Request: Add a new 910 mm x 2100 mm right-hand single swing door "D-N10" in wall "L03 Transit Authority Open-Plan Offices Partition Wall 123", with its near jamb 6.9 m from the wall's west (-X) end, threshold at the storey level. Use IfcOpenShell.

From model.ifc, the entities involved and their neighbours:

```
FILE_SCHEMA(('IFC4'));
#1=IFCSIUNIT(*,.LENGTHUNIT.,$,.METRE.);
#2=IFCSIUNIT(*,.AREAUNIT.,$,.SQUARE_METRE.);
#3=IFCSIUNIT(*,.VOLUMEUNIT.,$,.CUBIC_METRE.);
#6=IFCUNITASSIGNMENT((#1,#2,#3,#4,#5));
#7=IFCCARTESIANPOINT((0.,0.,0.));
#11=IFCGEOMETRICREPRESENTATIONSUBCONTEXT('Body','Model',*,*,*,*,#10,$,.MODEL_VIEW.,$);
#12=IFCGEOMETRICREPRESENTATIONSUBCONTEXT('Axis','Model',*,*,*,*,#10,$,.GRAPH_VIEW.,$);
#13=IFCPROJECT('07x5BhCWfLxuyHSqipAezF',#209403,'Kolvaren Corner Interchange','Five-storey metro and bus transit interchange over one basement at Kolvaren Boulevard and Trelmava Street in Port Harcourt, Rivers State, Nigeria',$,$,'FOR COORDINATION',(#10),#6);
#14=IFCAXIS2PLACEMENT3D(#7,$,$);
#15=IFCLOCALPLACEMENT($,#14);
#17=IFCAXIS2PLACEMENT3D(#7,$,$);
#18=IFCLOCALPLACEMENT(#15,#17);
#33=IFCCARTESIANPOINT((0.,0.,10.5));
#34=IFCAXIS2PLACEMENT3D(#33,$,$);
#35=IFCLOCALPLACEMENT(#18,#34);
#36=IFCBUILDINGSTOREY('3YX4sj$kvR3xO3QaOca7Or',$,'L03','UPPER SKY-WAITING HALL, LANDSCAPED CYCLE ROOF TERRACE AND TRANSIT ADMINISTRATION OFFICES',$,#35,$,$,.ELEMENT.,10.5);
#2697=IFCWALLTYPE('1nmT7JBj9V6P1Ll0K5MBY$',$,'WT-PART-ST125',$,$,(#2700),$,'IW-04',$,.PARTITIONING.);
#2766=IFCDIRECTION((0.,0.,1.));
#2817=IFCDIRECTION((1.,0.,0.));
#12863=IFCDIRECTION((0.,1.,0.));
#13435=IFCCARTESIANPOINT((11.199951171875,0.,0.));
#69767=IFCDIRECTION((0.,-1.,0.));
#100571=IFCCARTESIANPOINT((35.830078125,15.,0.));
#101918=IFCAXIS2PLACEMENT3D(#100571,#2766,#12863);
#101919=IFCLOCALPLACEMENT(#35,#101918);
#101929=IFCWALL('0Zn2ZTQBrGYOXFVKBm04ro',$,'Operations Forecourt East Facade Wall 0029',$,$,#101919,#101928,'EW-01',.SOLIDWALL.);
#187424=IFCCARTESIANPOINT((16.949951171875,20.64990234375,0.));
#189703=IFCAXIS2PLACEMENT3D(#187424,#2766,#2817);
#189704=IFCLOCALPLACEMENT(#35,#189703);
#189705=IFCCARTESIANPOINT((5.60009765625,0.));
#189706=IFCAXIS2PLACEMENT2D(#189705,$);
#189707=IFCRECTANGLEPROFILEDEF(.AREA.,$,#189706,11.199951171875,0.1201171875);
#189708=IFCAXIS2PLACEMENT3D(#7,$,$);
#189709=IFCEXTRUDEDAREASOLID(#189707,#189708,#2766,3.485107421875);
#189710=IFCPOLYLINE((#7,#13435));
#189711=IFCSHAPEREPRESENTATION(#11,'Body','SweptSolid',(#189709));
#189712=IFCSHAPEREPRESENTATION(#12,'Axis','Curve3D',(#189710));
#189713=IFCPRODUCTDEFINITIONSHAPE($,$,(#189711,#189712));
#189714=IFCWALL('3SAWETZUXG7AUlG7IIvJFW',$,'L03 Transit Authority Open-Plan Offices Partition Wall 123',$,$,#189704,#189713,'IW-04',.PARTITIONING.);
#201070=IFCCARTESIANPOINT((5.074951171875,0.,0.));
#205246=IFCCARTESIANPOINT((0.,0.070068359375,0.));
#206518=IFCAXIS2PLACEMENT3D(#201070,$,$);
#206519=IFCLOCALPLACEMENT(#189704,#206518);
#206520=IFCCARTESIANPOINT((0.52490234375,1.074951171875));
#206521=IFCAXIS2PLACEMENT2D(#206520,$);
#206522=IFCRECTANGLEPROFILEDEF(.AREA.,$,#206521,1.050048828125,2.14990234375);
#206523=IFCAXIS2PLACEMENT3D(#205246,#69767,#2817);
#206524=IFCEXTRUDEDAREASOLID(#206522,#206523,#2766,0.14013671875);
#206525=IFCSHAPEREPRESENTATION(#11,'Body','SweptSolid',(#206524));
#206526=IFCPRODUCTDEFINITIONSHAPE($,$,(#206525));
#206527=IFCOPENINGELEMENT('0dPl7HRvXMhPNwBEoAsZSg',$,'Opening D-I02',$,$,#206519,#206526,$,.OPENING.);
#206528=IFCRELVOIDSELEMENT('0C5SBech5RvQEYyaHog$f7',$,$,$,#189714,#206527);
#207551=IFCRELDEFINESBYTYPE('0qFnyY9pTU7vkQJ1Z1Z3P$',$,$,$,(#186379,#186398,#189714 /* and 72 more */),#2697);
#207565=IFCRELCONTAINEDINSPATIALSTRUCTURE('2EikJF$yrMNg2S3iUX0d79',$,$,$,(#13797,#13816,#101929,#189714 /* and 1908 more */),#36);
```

```python
import numpy as np
import ifcopenshell
import ifcopenshell.api.feature
import ifcopenshell.api.geometry
import ifcopenshell.api.root
import ifcopenshell.api.spatial
import ifcopenshell.geom
import ifcopenshell.util.element
import ifcopenshell.util.placement
import ifcopenshell.util.representation
import ifcopenshell.util.shape
import ifcopenshell.util.unit

model = ifcopenshell.open("model.ifc")
unit_scale = ifcopenshell.util.unit.calculate_unit_scale(model)
settings = ifcopenshell.geom.settings()


def volume(element):
    """Net volume in cubic metres, openings subtracted."""
    shape = ifcopenshell.geom.create_shape(settings, element)
    return ifcopenshell.util.shape.get_volume(shape.geometry)


wall = model.by_guid("3SAWETZUXG7AUlG7IIvJFW")
storey = ifcopenshell.util.element.get_container(wall, ifc_class="IfcBuildingStorey")
context = ifcopenshell.util.representation.get_context(model, "Model", "Body", "MODEL_VIEW")
before = volume(wall)

width, height, from_end, sill = 0.91, 2.1, 6.9, 0.0  # metres

# The wall runs along its own X axis, and the end named is its -X end.
wall_shape = ifcopenshell.geom.create_shape(settings, wall)
x, y, z = ifcopenshell.util.shape.get_vertices(wall_shape.geometry).T
start = x.min() + from_end
face, thickness = float(y.min()), float(y.max() - y.min())
wall_matrix = ifcopenshell.util.placement.get_local_placement(wall.ObjectPlacement)
level = ifcopenshell.util.placement.get_local_placement(storey.ObjectPlacement)[2, 3]


def in_wall(x, y):
    """Placement at x, y metres in the wall's axes, at sill height."""
    matrix = wall_matrix.copy()
    matrix[:, 3] = wall_matrix @ np.array([x / unit_scale, y / unit_scale, 0.0, 1.0])
    matrix[2, 3] = level + sill / unit_scale
    return matrix


# Opening: a box that overshoots both wall faces by 50 mm.
opening = ifcopenshell.api.root.create_entity(model, ifc_class="IfcOpeningElement", predefined_type="OPENING")
box = ifcopenshell.api.geometry.add_wall_representation(
    model, context=context, length=width, height=height, thickness=thickness + 0.1
)
ifcopenshell.api.geometry.assign_representation(model, product=opening, representation=box)
ifcopenshell.api.geometry.edit_object_placement(model, product=opening, matrix=in_wall(start, face - 0.05), is_si=False)
ifcopenshell.api.feature.add_feature(model, feature=opening, element=wall)

door = ifcopenshell.api.root.create_entity(model, ifc_class="IfcDoor", name="D-N10", predefined_type="DOOR")
door.OverallWidth, door.OverallHeight = width / unit_scale, height / unit_scale
door.OperationType = "SINGLE_SWING_RIGHT"
body = ifcopenshell.api.geometry.add_door_representation(
    model,
    context=context,
    overall_width=door.OverallWidth,
    overall_height=door.OverallHeight,
    operation_type="SINGLE_SWING_RIGHT",
    lining_properties={"LiningDepth": thickness / unit_scale, "ThresholdDepth": thickness / unit_scale},
)
ifcopenshell.api.geometry.assign_representation(model, product=door, representation=body)
ifcopenshell.api.spatial.assign_container(model, products=[door], relating_structure=storey)
ifcopenshell.api.feature.add_filling(model, opening=opening, element=door)

# The lining spans the wall, so the door starts at the wall face.
ifcopenshell.api.geometry.edit_object_placement(model, product=door, matrix=in_wall(start, face), is_si=False)

after = volume(wall)

print(f"wall volume {before:.3f} -> {after:.3f} m3")

model.write("model_rev.ifc")
```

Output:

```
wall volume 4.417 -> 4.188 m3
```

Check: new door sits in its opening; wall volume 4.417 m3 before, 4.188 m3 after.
